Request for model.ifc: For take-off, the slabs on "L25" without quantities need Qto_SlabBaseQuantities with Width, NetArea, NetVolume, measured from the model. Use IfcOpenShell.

First a look at what the model holds.

```python
import ifcopenshell
import ifcopenshell.util.element
import ifcopenshell.util.unit

model = ifcopenshell.open("model.ifc")
print(model.schema)
for unit_type in ("LENGTHUNIT", "AREAUNIT", "VOLUMEUNIT"):
    print(unit_type, ifcopenshell.util.unit.calculate_unit_scale(model, unit_type))
storey = next(s for s in model.by_type("IfcBuildingStorey") if s.Name == "L25")
slabs = [e for e in ifcopenshell.util.element.get_decomposition(storey) if e.is_a("IfcSlab")]
for e in sorted(slabs, key=lambda e: e.id()):
    print(e.id(), e.is_a(), e.Name, list(ifcopenshell.util.element.get_psets(e, qtos_only=True)), sep=" | ")
```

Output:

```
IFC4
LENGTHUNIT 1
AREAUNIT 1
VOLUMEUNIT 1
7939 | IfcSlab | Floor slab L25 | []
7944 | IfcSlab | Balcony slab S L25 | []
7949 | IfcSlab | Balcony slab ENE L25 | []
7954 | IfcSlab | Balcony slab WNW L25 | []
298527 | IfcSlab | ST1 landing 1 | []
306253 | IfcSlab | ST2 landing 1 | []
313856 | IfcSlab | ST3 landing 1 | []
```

```python
import ifcopenshell
import ifcopenshell.api.pset
import ifcopenshell.geom
import ifcopenshell.util.element
import ifcopenshell.util.shape
import ifcopenshell.util.unit

model = ifcopenshell.open("model.ifc")
unit_scale = ifcopenshell.util.unit.calculate_unit_scale(model)
area_scale = ifcopenshell.util.unit.calculate_unit_scale(model, "AREAUNIT")
volume_scale = ifcopenshell.util.unit.calculate_unit_scale(model, "VOLUMEUNIT")
settings = ifcopenshell.geom.settings()

storey = next(s for s in model.by_type("IfcBuildingStorey") if s.Name == "L25")
slabs = [e for e in ifcopenshell.util.element.get_decomposition(storey) if e.is_a("IfcSlab")]

for e in sorted(slabs, key=lambda e: e.id()):
    if ifcopenshell.util.element.get_psets(e, qtos_only=True, should_inherit=False):
        continue
    # Geometry comes back in metres, in the element's own axes.
    shape = ifcopenshell.geom.create_shape(settings, e)
    values = {
        "Width": ifcopenshell.util.shape.get_z(shape.geometry) / unit_scale,
        "NetArea": ifcopenshell.util.shape.get_footprint_area(shape.geometry) / area_scale,
        "NetVolume": ifcopenshell.util.shape.get_volume(shape.geometry) / volume_scale,
    }
    qto = ifcopenshell.api.pset.add_qto(model, product=e, name="Qto_SlabBaseQuantities")
    ifcopenshell.api.pset.edit_qto(model, qto=qto, properties=values)
    print(e.id(), {k: round(v, 3) for k, v in values.items()})

model.write("model_v2.ifc")
```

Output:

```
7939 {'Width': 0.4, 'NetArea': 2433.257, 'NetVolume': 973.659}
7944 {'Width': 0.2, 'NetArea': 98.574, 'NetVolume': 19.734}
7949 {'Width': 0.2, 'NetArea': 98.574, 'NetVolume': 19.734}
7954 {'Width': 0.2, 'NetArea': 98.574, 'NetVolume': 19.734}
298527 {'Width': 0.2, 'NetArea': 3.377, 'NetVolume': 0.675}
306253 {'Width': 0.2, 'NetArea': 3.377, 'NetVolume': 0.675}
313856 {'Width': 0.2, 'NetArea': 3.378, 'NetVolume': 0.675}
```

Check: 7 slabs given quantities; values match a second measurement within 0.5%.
